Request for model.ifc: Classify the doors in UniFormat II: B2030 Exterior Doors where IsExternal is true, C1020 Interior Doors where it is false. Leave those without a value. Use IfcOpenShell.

First a look at what the model holds.

```python
import ifcopenshell
import ifcopenshell.util.element

model = ifcopenshell.open("model.ifc")
print(model.schema)
print("classifications:", [c.Name for c in model.by_type("IfcClassification")])
values = [ifcopenshell.util.element.get_pset(e, "Pset_DoorCommon", "IsExternal") for e in model.by_type("IfcDoor")]
for value in (True, False, None):
    print("IsExternal", value, values.count(value))
```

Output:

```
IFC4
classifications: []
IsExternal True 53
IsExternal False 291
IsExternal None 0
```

```python
import ifcopenshell
import ifcopenshell.api.classification
import ifcopenshell.util.element

model = ifcopenshell.open("model.ifc")

system = ifcopenshell.api.classification.add_classification(model, classification="UniFormat II")

doors = model.by_type("IfcDoor")
external = {e: ifcopenshell.util.element.get_pset(e, "Pset_DoorCommon", "IsExternal") for e in doors}
for flag, code, name in ((True, "B2030", "Exterior Doors"), (False, "C1020", "Interior Doors")):
    products = [e for e in doors if external[e] is flag]
    ifcopenshell.api.classification.add_reference(
        model, products=products, classification=system, identification=code, name=name
    )
    print(code, len(products))

model.write("model_edited.ifc")
```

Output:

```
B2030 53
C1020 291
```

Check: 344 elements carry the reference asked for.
